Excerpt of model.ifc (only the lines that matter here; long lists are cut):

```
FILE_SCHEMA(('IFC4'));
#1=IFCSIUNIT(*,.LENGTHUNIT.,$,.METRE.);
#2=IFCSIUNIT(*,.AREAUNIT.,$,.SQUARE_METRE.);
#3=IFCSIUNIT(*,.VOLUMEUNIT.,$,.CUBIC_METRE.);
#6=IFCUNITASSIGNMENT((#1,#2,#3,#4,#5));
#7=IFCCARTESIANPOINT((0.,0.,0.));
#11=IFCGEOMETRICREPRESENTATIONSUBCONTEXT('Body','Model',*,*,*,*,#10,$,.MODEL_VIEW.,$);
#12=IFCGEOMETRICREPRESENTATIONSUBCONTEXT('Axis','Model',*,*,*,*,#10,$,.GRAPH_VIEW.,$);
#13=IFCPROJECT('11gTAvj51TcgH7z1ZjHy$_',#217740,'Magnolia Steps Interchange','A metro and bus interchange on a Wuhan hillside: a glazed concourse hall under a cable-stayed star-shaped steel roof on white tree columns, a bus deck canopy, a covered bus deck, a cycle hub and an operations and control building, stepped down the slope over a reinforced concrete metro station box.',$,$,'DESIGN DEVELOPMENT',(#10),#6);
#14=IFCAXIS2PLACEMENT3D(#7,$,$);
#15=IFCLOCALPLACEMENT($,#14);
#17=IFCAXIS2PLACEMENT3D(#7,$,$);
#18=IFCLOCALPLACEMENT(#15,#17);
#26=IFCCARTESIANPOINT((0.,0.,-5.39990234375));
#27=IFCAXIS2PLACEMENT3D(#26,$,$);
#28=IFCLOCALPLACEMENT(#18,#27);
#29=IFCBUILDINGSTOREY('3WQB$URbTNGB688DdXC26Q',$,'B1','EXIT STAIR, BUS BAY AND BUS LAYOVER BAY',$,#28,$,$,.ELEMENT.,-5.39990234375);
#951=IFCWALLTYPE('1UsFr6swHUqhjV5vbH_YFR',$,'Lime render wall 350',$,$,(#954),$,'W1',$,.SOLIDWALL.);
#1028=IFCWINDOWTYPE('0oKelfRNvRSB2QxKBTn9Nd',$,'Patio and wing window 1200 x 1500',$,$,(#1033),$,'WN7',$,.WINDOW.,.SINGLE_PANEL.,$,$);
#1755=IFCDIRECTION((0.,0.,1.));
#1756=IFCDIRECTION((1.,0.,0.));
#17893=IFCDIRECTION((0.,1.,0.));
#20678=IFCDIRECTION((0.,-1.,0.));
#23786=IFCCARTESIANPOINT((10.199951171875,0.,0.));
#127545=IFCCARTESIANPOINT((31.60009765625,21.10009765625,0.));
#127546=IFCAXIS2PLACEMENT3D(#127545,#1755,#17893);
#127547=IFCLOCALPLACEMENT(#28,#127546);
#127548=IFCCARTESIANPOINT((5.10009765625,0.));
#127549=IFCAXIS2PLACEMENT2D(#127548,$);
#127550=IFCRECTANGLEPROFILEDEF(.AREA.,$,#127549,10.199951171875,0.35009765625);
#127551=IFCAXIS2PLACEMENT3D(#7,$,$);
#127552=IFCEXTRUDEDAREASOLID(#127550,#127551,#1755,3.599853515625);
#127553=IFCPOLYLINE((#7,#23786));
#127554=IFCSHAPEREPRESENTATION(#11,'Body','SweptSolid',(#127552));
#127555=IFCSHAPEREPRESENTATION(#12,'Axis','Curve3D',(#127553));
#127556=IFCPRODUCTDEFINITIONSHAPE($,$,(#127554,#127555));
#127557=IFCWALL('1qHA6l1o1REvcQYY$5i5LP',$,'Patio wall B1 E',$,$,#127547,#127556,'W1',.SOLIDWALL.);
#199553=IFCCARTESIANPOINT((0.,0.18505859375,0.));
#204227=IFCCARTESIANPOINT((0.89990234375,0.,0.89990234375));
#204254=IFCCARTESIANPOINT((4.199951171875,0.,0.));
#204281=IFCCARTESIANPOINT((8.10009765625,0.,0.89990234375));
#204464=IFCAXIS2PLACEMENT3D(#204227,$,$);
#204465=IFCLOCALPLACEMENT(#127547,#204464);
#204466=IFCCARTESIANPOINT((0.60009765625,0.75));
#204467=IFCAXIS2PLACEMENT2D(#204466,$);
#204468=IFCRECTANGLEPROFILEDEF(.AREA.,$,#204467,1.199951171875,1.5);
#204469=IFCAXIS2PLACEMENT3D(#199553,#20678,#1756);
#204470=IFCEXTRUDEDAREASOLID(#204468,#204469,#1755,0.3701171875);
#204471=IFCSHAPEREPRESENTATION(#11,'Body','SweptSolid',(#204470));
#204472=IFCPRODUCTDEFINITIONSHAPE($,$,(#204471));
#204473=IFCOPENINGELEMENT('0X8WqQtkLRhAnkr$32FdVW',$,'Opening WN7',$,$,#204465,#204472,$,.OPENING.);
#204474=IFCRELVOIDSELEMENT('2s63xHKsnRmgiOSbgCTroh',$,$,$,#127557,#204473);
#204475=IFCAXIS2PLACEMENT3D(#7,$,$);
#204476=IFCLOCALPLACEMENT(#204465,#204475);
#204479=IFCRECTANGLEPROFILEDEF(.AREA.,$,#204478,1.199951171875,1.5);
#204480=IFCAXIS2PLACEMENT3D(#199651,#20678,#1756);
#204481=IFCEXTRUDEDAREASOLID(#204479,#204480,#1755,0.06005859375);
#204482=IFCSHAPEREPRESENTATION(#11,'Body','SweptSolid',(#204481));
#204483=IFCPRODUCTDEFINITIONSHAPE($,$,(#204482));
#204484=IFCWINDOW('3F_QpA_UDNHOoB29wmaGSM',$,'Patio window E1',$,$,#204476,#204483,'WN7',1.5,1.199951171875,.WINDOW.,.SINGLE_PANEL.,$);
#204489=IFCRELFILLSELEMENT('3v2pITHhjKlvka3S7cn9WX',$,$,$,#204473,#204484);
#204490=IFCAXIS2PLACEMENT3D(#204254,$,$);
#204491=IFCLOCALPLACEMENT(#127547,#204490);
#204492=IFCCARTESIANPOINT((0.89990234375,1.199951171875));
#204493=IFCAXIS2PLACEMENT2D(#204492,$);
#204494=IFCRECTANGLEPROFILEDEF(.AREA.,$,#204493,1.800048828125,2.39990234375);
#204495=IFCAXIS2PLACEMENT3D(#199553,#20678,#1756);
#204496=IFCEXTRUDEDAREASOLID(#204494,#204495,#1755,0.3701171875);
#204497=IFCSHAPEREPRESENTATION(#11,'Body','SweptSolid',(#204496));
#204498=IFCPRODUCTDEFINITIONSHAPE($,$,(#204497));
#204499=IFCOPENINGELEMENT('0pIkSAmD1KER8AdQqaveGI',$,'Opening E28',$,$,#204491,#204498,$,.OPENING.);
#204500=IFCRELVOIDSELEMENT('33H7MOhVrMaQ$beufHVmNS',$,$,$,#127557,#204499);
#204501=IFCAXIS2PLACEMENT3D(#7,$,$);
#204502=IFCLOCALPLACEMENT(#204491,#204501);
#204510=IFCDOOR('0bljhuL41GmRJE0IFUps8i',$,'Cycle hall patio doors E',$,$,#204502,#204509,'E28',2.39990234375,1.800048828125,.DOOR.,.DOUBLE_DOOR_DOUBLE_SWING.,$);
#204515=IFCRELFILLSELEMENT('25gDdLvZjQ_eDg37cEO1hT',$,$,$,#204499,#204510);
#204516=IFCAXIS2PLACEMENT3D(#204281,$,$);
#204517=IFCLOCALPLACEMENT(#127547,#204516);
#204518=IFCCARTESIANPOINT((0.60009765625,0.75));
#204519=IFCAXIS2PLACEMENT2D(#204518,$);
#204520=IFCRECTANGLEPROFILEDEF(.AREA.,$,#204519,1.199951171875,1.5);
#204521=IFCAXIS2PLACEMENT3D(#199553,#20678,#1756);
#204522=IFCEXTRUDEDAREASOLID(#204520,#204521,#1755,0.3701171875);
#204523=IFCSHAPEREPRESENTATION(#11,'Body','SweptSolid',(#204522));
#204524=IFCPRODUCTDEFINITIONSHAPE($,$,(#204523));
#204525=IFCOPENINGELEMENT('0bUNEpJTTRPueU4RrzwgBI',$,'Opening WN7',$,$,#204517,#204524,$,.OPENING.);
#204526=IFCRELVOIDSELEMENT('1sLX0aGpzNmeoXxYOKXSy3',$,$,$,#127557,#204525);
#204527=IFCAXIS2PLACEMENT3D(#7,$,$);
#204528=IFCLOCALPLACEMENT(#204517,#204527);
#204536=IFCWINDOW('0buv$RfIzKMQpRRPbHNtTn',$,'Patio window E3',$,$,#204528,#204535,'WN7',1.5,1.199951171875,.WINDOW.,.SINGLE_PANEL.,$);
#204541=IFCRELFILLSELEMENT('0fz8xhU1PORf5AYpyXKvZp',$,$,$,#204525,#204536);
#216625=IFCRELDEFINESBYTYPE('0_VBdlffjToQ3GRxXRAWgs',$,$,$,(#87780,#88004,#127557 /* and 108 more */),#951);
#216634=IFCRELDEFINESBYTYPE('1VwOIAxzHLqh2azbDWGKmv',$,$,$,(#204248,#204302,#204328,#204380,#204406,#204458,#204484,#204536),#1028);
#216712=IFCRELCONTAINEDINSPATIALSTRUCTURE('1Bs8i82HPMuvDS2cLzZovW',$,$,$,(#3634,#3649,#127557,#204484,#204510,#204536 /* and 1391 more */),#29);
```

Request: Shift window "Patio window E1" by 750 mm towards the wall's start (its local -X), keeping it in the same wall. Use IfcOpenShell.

```python
import ifcopenshell
import ifcopenshell.api.geometry
import ifcopenshell.util.placement
import ifcopenshell.util.unit

model = ifcopenshell.open("model.ifc")
unit_scale = ifcopenshell.util.unit.calculate_unit_scale(model)

window = model.by_id(204484)
opening = window.FillsVoids[0].RelatingOpeningElement
wall = opening.VoidsElements[0].RelatingBuildingElement

wall_matrix = ifcopenshell.util.placement.get_local_placement(wall.ObjectPlacement)
shift = wall_matrix[:3, 0] * -0.75 / unit_scale
before = ifcopenshell.util.placement.get_local_placement(window.ObjectPlacement)[:3, 3].copy()

# The window is placed relative to its opening, so it follows when the opening moves.
matrix = ifcopenshell.util.placement.get_local_placement(opening.ObjectPlacement)
matrix[:3, 3] += shift
ifcopenshell.api.geometry.edit_object_placement(
    model, product=opening, matrix=matrix, is_si=False, should_transform_children=True
)

after = ifcopenshell.util.placement.get_local_placement(window.ObjectPlacement)[:3, 3]
print("window moved by", (after - before).round(3) + 0.0)

model.write("model_rev.ifc")
```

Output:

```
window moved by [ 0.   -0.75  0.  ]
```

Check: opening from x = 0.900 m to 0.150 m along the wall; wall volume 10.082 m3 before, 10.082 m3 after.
